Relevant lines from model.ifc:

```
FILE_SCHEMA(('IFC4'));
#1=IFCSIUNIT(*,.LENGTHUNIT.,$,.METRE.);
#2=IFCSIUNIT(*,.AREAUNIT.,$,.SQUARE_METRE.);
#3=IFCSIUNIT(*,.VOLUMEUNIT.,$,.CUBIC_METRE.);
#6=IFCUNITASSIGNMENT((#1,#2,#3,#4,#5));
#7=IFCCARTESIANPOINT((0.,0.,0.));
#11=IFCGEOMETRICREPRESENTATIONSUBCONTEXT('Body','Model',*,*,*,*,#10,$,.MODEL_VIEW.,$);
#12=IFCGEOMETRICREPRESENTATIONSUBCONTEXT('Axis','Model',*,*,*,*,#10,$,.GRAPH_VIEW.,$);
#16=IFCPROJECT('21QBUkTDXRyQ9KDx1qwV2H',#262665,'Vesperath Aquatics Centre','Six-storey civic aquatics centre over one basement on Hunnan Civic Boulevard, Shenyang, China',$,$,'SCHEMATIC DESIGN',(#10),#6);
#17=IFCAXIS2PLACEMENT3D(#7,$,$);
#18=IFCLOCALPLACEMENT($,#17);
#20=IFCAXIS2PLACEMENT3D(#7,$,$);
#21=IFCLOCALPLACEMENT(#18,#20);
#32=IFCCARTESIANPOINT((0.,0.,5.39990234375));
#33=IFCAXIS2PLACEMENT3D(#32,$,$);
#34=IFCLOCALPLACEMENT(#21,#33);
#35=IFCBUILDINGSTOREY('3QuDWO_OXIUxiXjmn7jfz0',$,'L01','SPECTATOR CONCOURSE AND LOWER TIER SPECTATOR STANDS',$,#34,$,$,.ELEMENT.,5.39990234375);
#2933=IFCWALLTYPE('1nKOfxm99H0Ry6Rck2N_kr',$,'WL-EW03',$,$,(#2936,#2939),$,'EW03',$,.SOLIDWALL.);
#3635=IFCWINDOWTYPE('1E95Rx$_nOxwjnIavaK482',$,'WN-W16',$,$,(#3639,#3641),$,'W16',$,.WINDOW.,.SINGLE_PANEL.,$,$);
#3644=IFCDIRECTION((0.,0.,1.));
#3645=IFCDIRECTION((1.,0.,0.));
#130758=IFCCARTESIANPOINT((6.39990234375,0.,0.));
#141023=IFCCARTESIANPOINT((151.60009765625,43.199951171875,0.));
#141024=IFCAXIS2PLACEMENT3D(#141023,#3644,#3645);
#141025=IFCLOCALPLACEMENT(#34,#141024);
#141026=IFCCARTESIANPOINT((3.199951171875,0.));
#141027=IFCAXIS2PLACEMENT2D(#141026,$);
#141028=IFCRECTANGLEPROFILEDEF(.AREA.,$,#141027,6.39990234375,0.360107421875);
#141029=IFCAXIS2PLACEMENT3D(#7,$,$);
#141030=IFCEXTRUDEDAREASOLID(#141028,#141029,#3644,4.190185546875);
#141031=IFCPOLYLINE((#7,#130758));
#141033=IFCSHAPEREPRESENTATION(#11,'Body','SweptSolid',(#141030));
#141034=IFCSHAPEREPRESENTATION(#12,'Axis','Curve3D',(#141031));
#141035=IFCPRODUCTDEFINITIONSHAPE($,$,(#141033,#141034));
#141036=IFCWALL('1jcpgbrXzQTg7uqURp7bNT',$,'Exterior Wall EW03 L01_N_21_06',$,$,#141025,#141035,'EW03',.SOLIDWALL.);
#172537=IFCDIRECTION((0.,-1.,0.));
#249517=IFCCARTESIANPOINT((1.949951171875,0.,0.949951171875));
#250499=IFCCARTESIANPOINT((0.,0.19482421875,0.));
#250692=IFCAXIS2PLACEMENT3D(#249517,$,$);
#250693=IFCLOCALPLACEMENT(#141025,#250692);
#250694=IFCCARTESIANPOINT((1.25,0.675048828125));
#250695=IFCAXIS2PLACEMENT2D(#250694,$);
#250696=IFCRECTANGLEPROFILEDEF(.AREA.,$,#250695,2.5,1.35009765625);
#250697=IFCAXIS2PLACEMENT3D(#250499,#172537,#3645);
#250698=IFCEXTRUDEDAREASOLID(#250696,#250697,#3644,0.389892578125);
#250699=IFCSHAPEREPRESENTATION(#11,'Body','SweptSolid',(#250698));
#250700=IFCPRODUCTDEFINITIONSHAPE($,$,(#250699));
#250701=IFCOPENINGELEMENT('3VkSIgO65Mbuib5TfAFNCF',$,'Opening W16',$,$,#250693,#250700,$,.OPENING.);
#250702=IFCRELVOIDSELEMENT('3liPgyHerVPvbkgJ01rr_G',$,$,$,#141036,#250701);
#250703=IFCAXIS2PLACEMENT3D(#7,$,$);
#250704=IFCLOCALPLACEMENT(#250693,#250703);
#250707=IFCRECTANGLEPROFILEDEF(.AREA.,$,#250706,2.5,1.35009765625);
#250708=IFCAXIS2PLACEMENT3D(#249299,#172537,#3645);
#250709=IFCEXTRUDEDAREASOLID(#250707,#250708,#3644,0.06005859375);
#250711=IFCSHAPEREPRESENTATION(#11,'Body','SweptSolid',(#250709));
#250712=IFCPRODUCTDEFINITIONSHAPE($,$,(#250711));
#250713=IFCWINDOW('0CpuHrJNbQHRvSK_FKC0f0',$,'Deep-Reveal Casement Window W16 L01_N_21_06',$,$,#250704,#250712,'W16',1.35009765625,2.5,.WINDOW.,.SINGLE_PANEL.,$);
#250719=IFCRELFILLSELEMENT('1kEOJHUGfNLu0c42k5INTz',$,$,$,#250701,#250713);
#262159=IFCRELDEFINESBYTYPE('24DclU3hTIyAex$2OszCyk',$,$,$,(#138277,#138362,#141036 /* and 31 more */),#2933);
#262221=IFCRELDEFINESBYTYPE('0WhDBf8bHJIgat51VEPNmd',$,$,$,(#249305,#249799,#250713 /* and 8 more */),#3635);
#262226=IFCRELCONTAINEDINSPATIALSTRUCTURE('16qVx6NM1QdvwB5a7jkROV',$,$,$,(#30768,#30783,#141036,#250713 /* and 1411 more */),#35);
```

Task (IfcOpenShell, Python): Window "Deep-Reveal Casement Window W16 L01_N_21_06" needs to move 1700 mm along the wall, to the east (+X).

```python
import ifcopenshell
import ifcopenshell.api.geometry
import ifcopenshell.util.placement

model = ifcopenshell.open("model.ifc")

window = model.by_guid("0CpuHrJNbQHRvSK_FKC0f0")
opening = window.FillsVoids[0].RelatingOpeningElement
wall = opening.VoidsElements[0].RelatingBuildingElement

wall_matrix = ifcopenshell.util.placement.get_local_placement(wall.ObjectPlacement)
shift = wall_matrix[:3, 0] * 1.7
before = ifcopenshell.util.placement.get_local_placement(window.ObjectPlacement)[:3, 3].copy()

# The window is placed relative to its opening, so it follows when the opening moves.
matrix = ifcopenshell.util.placement.get_local_placement(opening.ObjectPlacement)
matrix[:3, 3] += shift
ifcopenshell.api.geometry.edit_object_placement(
    model, product=opening, matrix=matrix, is_si=False, should_transform_children=True
)

after = ifcopenshell.util.placement.get_local_placement(window.ObjectPlacement)[:3, 3]
print("window moved by", (after - before).round(3) + 0.0)

model.write("model_v2.ifc")
```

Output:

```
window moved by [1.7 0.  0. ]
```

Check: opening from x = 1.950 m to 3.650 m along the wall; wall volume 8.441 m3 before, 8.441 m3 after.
